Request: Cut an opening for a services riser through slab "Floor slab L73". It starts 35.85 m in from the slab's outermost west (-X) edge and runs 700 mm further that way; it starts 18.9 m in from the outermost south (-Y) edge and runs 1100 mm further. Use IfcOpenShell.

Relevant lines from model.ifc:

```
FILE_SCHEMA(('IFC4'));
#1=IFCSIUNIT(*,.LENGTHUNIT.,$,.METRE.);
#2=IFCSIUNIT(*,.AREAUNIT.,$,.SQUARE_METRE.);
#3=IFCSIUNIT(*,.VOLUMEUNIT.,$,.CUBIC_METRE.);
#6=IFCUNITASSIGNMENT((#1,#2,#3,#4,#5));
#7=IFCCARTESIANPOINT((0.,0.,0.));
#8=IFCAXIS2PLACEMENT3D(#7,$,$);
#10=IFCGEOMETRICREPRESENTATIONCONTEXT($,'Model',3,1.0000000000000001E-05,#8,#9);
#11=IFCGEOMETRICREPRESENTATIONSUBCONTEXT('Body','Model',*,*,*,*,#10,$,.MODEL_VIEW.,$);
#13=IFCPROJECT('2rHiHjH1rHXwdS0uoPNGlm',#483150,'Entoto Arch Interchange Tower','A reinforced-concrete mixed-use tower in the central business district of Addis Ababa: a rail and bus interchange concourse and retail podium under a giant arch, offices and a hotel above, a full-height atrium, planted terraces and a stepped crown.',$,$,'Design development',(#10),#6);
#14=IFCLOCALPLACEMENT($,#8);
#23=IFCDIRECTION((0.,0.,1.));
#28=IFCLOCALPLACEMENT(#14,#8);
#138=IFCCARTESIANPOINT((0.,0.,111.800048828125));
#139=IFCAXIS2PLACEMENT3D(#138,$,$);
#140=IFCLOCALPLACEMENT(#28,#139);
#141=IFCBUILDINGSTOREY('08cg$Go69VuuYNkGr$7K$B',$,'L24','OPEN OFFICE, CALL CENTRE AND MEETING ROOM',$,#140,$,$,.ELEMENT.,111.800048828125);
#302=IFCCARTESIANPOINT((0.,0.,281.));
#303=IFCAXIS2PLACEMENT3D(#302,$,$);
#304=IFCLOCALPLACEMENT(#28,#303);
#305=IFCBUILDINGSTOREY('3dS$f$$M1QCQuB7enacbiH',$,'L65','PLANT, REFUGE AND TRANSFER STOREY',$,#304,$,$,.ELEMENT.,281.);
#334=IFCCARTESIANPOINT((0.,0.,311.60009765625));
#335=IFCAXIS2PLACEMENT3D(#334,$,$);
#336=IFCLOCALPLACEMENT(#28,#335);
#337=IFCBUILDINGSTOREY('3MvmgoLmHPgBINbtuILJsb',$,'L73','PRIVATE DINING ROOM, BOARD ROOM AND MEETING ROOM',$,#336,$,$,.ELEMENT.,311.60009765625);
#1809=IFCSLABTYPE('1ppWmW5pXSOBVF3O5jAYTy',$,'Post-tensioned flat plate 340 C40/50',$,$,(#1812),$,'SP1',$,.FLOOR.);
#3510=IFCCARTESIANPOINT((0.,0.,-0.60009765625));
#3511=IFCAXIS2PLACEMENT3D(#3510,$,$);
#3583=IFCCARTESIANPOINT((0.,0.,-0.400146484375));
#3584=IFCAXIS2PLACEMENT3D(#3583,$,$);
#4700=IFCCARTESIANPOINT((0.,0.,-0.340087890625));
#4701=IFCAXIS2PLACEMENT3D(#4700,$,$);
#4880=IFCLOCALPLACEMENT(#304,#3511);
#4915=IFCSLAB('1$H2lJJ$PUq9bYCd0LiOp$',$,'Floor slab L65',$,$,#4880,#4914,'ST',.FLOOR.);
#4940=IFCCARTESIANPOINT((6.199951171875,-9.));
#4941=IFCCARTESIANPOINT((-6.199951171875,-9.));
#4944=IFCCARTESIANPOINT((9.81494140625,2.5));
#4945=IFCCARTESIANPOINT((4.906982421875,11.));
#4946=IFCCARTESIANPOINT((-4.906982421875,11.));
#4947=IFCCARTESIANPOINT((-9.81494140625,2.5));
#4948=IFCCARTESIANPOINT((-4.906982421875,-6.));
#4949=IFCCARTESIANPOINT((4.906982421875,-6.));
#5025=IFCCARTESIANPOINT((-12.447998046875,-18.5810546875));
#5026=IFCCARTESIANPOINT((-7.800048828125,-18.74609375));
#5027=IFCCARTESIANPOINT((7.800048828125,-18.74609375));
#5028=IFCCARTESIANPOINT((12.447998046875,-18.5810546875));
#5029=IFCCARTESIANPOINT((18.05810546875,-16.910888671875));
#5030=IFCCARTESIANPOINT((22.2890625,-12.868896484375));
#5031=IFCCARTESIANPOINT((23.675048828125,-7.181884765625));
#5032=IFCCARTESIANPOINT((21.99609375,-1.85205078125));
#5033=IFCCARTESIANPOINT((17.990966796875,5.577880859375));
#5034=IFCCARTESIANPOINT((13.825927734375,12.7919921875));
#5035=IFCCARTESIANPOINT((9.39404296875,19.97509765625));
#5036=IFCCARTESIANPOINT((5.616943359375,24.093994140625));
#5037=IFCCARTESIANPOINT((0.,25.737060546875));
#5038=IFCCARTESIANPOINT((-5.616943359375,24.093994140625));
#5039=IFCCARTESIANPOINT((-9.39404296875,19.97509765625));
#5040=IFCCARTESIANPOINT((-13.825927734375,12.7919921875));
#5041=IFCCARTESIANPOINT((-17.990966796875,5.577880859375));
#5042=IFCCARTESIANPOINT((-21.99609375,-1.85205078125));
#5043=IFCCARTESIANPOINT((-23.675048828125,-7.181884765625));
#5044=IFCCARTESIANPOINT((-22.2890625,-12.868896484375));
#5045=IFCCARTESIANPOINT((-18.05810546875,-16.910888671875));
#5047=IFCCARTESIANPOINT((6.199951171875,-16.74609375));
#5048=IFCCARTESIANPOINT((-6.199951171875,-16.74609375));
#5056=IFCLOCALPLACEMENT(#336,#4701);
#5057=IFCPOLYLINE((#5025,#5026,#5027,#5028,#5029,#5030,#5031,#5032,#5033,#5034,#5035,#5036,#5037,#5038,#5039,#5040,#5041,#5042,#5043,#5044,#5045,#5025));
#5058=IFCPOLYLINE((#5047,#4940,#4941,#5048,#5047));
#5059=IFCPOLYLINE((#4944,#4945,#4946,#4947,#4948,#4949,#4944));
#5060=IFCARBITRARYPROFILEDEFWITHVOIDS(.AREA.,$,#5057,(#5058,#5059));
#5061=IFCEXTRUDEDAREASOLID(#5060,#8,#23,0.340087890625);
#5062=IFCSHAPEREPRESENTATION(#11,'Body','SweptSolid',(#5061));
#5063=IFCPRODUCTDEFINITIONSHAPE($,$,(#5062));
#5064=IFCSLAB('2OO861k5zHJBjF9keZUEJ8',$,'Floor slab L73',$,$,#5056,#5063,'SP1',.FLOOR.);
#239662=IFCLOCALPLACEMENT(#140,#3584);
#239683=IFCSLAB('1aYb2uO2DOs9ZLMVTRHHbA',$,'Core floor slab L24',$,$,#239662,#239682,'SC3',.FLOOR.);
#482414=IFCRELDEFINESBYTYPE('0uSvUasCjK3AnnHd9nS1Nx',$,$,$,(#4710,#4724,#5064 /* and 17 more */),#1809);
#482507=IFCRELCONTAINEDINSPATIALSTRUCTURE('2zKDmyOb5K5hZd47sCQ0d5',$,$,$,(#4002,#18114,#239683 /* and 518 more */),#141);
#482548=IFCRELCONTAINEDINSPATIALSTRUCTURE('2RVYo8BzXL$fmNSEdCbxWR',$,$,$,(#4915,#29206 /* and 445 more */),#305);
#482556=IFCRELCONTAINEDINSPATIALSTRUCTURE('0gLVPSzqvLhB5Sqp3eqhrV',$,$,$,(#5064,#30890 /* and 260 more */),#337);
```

```python
import numpy as np
import ifcopenshell
import ifcopenshell.api.feature
import ifcopenshell.api.geometry
import ifcopenshell.api.root
import ifcopenshell.geom
import ifcopenshell.util.placement
import ifcopenshell.util.representation
import ifcopenshell.util.shape
import ifcopenshell.util.unit

model = ifcopenshell.open("model.ifc")
unit_scale = ifcopenshell.util.unit.calculate_unit_scale(model)
settings = ifcopenshell.geom.settings()


def volume(element):
    """Net volume in cubic metres, openings subtracted."""
    shape = ifcopenshell.geom.create_shape(settings, element)
    return ifcopenshell.util.shape.get_volume(shape.geometry)


slab = model.by_id(5064)
before = volume(slab)

# Extent in the slab's own axes, in metres. The edges named are its -X and -Y sides.
slab_shape = ifcopenshell.geom.create_shape(settings, slab)
vertices = ifcopenshell.util.shape.get_vertices(slab_shape.geometry)
x_min, y_min, bottom = vertices.min(axis=0)
top = vertices[:, 2].max()

opening = ifcopenshell.api.root.create_entity(model, ifc_class="IfcOpeningElement", name="Services riser opening", predefined_type="OPENING")
context = ifcopenshell.util.representation.get_context(model, "Model", "Body", "MODEL_VIEW")
width, depth = 0.7, 1.1
outline = [(0.0, 0.0), (width, 0.0), (width, depth), (0.0, depth), (0.0, 0.0)]
# Overshoot both faces by 50 mm so the cut is clean.
shape = ifcopenshell.api.geometry.add_slab_representation(
    model, context=context, depth=top - bottom + 0.1, polyline=outline
)
ifcopenshell.api.geometry.assign_representation(model, product=opening, representation=shape)

matrix = ifcopenshell.util.placement.get_local_placement(slab.ObjectPlacement)
matrix[:, 3] = matrix @ np.append(np.array([x_min + 35.85, y_min + 18.9, bottom - 0.05]) / unit_scale, 1.0)
ifcopenshell.api.geometry.edit_object_placement(model, product=opening, matrix=matrix, is_si=False)
ifcopenshell.api.feature.add_feature(model, feature=opening, element=slab)

after = volume(slab)

print(f"slab volume {before:.3f} -> {after:.3f} m3")

model.write("model-out.ifc")
```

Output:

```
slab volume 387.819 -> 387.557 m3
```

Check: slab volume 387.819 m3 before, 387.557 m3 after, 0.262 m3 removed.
